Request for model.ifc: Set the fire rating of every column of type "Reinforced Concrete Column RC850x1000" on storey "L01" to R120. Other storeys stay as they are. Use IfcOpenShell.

First a look at what the model holds.

```python
import ifcopenshell
import ifcopenshell.util.element

model = ifcopenshell.open("model.ifc")
print(model.schema)
storey = next(s for s in model.by_type("IfcBuildingStorey") if s.Name == "L01")
columns = [e for e in ifcopenshell.util.element.get_decomposition(storey) if e.is_a("IfcColumn")]
seen = {}
for e in columns:
    element_type = ifcopenshell.util.element.get_type(e)
    key = (element_type.Name if element_type != e and element_type else None, ifcopenshell.util.element.get_pset(e, "Pset_ColumnCommon", "FireRating"))
    seen[key] = seen.get(key, 0) + 1
for (name, value), count in sorted(seen.items(), key=str):
    print(count, "x", name, "|", value)
```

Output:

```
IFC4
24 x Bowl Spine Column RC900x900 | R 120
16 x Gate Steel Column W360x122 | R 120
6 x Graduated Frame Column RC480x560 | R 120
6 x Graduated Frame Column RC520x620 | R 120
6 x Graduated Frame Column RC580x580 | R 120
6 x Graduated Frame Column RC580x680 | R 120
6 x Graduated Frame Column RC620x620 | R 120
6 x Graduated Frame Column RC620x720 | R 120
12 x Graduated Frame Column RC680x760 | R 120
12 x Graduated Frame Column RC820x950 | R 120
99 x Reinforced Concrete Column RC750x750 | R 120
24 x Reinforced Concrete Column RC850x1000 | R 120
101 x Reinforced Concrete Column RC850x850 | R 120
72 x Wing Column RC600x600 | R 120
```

```python
import ifcopenshell
import ifcopenshell.api.pset
import ifcopenshell.util.element

model = ifcopenshell.open("model.ifc")

storey = next(s for s in model.by_type("IfcBuildingStorey") if s.Name == "L01")
columns = [e for e in ifcopenshell.util.element.get_decomposition(storey) if e.is_a("IfcColumn")]

count = 0
for e in columns:
    element_type = ifcopenshell.util.element.get_type(e)
    if element_type in (None, e) or element_type.Name != "Reinforced Concrete Column RC850x1000":
        continue
    # add_pset returns the element's existing set when there is one.
    pset = ifcopenshell.api.pset.add_pset(model, product=e, name="Pset_ColumnCommon")
    ifcopenshell.api.pset.edit_pset(model, pset=pset, properties={"FireRating": "R120"})
    count += 1

print(count, "columns updated")

model.write("model-out.ifc")
```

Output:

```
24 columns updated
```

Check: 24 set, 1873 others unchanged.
